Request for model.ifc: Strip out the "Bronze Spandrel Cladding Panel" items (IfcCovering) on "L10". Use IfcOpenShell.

First a look at what the model holds.

```python
import ifcopenshell
import ifcopenshell.util.element

model = ifcopenshell.open("model.ifc")
print(model.schema)
storey = next(s for s in model.by_type("IfcBuildingStorey") if s.Name == "L10")
coverings = [e for e in ifcopenshell.util.element.get_decomposition(storey) if e.is_a("IfcCovering")]
seen = {}
for e in coverings:
    element_type = ifcopenshell.util.element.get_type(e)
    name = element_type.Name if element_type not in (None, e) else None
    seen[name] = seen.get(name, 0) + 1
for name, count in sorted(seen.items(), key=str):
    print(count, "x", name)
```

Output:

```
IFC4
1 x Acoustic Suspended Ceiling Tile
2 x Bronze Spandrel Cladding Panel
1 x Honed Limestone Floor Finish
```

```python
import ifcopenshell
import ifcopenshell.api.root
import ifcopenshell.util.element

model = ifcopenshell.open("model.ifc")

storey = next(s for s in model.by_type("IfcBuildingStorey") if s.Name == "L10")
coverings = [e for e in ifcopenshell.util.element.get_decomposition(storey) if e.is_a("IfcCovering")]
targets = [e for e in coverings if (t := ifcopenshell.util.element.get_type(e)) not in (None, e) and t.Name == "Bronze Spandrel Cladding Panel"]

for e in targets:
    ifcopenshell.api.root.remove_product(model, product=e)
print(len(targets), "removed")

model.write("model_edited.ifc")
```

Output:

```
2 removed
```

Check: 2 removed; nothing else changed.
